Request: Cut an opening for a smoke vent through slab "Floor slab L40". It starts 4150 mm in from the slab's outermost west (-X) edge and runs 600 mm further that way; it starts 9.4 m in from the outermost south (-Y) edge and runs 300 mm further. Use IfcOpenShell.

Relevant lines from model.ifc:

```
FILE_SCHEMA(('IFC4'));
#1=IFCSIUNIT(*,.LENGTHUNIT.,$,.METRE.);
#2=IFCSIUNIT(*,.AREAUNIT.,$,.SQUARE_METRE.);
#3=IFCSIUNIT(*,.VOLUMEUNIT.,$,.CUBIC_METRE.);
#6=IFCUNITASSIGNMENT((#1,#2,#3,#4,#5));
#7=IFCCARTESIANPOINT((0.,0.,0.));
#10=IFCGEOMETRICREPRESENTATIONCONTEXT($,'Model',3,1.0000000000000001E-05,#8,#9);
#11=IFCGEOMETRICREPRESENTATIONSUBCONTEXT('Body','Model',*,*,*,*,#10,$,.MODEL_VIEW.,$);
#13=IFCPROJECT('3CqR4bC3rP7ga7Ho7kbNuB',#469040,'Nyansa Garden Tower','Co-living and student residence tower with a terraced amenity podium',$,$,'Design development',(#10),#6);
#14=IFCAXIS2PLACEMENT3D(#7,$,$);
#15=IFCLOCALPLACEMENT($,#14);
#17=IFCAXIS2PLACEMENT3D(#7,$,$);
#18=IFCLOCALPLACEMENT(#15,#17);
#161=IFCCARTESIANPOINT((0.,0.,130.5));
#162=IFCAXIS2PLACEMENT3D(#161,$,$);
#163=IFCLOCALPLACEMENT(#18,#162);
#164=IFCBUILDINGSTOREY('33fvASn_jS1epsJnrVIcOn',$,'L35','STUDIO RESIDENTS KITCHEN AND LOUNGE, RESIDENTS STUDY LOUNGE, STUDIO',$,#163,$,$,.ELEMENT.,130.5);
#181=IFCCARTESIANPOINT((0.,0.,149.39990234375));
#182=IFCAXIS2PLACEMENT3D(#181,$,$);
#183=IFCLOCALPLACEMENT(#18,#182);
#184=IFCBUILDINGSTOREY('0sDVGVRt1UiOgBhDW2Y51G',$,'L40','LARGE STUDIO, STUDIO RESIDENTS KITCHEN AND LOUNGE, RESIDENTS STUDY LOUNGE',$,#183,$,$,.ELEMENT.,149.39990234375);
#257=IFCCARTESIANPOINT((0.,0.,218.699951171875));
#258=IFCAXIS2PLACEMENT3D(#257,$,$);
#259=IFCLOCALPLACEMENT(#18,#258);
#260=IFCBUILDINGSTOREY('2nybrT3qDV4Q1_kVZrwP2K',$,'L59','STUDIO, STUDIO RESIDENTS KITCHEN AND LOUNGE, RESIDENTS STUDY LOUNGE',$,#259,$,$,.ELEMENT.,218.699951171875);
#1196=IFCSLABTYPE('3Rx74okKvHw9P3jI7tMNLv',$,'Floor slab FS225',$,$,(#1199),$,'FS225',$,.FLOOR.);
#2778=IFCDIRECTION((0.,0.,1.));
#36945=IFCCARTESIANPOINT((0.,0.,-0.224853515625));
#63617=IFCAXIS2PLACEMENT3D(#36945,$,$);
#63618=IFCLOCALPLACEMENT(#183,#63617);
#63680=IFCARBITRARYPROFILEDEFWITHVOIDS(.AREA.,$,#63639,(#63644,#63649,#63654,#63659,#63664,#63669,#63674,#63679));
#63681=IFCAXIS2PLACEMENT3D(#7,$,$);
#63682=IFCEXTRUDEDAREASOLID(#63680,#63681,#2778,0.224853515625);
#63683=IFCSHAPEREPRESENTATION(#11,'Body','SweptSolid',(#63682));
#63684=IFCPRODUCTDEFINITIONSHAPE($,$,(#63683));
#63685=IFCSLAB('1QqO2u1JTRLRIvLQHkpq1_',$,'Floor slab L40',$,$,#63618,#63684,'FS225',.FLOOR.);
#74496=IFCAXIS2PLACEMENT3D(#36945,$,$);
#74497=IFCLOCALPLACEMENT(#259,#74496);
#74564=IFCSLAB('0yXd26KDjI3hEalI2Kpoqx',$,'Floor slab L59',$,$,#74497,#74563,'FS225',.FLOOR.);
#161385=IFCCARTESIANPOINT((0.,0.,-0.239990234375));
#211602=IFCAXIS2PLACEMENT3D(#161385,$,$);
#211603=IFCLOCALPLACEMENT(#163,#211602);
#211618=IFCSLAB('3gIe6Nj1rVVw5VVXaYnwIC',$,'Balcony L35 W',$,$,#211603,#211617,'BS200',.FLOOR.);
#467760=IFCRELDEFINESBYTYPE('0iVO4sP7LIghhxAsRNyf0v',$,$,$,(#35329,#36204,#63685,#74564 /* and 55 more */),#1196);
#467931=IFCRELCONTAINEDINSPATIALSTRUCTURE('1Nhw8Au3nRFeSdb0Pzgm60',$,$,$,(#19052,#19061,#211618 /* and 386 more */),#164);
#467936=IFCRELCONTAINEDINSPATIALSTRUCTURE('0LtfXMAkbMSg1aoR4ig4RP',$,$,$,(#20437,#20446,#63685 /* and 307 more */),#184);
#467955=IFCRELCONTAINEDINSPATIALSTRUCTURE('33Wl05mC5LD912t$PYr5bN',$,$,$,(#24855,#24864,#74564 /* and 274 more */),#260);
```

```python
import numpy as np
import ifcopenshell
import ifcopenshell.api.feature
import ifcopenshell.api.geometry
import ifcopenshell.api.root
import ifcopenshell.geom
import ifcopenshell.util.placement
import ifcopenshell.util.representation
import ifcopenshell.util.shape
import ifcopenshell.util.unit

model = ifcopenshell.open("model.ifc")
unit_scale = ifcopenshell.util.unit.calculate_unit_scale(model)
settings = ifcopenshell.geom.settings()


def volume(element):
    """Net volume in cubic metres, openings subtracted."""
    shape = ifcopenshell.geom.create_shape(settings, element)
    return ifcopenshell.util.shape.get_volume(shape.geometry)


slab = model.by_id(63685)
before = volume(slab)

# Extent in the slab's own axes, in metres. The edges named are its -X and -Y sides.
slab_shape = ifcopenshell.geom.create_shape(settings, slab)
vertices = ifcopenshell.util.shape.get_vertices(slab_shape.geometry)
x_min, y_min, bottom = vertices.min(axis=0)
top = vertices[:, 2].max()

opening = ifcopenshell.api.root.create_entity(model, ifc_class="IfcOpeningElement", name="Smoke vent opening", predefined_type="OPENING")
context = ifcopenshell.util.representation.get_context(model, "Model", "Body", "MODEL_VIEW")
width, depth = 0.6, 0.3
outline = [(0.0, 0.0), (width, 0.0), (width, depth), (0.0, depth), (0.0, 0.0)]
# Overshoot both faces by 50 mm so the cut is clean.
shape = ifcopenshell.api.geometry.add_slab_representation(
    model, context=context, depth=top - bottom + 0.1, polyline=outline
)
ifcopenshell.api.geometry.assign_representation(model, product=opening, representation=shape)

matrix = ifcopenshell.util.placement.get_local_placement(slab.ObjectPlacement)
matrix[:, 3] = matrix @ np.append(np.array([x_min + 4.15, y_min + 9.4, bottom - 0.05]) / unit_scale, 1.0)
ifcopenshell.api.geometry.edit_object_placement(model, product=opening, matrix=matrix, is_si=False)
ifcopenshell.api.feature.add_feature(model, feature=opening, element=slab)

after = volume(slab)

print(f"slab volume {before:.3f} -> {after:.3f} m3")

model.write("model_updated.ifc")
```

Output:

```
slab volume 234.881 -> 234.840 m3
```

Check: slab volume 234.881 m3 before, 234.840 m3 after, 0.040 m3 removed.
